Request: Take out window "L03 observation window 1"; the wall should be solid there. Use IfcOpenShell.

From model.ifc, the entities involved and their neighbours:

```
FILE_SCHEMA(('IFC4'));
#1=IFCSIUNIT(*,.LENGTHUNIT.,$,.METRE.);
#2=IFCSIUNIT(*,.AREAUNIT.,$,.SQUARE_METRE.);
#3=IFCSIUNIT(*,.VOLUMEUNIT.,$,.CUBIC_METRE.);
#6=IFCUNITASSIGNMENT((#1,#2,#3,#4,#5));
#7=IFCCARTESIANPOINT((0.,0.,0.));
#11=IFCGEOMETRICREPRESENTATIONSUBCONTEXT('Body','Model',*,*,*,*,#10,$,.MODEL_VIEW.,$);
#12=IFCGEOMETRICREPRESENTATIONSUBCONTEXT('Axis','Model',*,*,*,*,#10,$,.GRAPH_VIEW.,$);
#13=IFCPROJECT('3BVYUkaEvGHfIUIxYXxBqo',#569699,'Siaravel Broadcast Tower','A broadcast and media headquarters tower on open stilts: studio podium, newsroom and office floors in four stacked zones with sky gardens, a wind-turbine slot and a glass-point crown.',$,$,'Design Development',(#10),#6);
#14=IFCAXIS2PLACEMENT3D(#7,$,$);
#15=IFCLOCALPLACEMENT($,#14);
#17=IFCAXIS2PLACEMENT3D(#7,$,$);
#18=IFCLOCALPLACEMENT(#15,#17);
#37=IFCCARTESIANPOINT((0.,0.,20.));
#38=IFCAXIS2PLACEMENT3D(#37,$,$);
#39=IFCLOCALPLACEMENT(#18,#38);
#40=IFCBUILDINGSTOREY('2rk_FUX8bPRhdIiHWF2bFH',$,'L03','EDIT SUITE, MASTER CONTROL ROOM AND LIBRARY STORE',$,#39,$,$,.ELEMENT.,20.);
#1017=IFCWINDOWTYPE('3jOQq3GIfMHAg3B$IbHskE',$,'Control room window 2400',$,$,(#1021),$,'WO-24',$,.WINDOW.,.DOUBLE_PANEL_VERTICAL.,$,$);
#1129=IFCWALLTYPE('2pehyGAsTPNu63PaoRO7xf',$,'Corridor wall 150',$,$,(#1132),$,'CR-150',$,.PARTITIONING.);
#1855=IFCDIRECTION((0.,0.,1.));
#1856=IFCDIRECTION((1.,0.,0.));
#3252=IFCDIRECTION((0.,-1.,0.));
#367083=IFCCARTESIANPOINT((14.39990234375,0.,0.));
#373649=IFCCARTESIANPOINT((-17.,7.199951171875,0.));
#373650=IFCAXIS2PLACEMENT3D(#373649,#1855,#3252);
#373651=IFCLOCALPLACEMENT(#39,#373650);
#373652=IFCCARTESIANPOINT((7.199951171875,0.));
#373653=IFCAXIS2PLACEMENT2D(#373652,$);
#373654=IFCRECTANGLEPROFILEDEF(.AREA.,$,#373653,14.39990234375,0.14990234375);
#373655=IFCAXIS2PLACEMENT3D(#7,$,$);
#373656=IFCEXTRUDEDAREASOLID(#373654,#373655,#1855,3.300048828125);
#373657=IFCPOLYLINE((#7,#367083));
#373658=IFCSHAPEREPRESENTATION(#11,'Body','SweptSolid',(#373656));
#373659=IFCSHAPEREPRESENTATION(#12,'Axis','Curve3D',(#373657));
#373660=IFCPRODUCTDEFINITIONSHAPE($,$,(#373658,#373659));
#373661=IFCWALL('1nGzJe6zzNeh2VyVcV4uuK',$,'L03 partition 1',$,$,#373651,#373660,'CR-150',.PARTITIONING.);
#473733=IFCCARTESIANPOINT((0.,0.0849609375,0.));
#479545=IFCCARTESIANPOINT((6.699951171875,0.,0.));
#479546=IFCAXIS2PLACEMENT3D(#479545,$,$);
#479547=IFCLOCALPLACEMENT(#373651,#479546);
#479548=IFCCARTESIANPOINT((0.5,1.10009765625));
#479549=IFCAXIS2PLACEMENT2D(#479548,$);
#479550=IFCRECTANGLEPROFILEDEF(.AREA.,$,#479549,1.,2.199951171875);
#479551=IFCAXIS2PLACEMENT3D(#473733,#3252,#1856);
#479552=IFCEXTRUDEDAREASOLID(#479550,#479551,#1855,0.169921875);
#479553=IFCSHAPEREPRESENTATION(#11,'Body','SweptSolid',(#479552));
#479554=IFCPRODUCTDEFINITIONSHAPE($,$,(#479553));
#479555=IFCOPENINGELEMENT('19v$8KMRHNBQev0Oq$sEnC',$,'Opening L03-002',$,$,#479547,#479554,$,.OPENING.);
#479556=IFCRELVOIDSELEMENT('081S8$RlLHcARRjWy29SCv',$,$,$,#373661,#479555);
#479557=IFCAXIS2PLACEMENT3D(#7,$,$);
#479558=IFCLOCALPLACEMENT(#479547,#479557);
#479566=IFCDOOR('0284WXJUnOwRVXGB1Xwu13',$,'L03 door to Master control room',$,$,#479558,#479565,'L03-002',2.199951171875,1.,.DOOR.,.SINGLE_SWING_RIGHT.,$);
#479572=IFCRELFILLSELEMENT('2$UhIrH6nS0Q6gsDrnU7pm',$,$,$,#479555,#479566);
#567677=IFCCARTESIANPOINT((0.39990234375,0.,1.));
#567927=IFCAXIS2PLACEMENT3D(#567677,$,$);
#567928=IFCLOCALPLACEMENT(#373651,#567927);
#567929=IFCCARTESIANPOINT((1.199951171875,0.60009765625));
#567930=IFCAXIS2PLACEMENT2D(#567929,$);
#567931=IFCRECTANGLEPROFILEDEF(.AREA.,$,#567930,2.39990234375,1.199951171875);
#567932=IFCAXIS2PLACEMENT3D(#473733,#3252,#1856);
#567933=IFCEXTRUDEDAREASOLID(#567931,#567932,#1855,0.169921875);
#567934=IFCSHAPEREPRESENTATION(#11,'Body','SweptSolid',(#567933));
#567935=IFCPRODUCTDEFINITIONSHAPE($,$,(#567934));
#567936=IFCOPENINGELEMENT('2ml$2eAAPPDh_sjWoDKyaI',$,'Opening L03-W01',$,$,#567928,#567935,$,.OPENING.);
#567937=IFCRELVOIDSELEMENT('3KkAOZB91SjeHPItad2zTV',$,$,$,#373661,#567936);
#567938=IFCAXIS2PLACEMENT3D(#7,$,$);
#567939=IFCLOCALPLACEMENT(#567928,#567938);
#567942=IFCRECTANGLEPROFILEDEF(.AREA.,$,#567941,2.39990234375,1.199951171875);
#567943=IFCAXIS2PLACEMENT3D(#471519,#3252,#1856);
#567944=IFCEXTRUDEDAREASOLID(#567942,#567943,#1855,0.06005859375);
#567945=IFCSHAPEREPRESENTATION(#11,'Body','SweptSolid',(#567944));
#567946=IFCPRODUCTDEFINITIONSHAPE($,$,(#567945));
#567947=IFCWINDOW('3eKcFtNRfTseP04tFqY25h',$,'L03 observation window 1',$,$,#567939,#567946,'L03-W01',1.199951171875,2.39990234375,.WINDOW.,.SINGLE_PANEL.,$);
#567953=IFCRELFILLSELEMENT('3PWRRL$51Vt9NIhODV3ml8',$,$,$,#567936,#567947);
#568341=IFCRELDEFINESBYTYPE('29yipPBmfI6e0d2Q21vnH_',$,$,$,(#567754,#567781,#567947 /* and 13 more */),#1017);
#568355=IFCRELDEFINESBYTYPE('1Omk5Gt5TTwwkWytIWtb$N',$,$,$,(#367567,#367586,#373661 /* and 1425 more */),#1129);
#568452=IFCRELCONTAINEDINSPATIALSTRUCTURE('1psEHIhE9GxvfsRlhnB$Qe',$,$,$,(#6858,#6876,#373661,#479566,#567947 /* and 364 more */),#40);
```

```python
import ifcopenshell
import ifcopenshell.api.feature
import ifcopenshell.api.root
import ifcopenshell.geom
import ifcopenshell.util.shape

model = ifcopenshell.open("model.ifc")
settings = ifcopenshell.geom.settings()


def volume(element):
    """Net volume in cubic metres, openings subtracted."""
    shape = ifcopenshell.geom.create_shape(settings, element)
    return ifcopenshell.util.shape.get_volume(shape.geometry)


window = model.by_guid("3eKcFtNRfTseP04tFqY25h")
opening = window.FillsVoids[0].RelatingOpeningElement
wall = opening.VoidsElements[0].RelatingBuildingElement
before = volume(wall)

ifcopenshell.api.root.remove_product(model, product=window)
ifcopenshell.api.feature.remove_feature(model, feature=opening)

after = volume(wall)

print(f"wall volume {before:.3f} -> {after:.3f} m3")

model.write("model_edited.ifc")
```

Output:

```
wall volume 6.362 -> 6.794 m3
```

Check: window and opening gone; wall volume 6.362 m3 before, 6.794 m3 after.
